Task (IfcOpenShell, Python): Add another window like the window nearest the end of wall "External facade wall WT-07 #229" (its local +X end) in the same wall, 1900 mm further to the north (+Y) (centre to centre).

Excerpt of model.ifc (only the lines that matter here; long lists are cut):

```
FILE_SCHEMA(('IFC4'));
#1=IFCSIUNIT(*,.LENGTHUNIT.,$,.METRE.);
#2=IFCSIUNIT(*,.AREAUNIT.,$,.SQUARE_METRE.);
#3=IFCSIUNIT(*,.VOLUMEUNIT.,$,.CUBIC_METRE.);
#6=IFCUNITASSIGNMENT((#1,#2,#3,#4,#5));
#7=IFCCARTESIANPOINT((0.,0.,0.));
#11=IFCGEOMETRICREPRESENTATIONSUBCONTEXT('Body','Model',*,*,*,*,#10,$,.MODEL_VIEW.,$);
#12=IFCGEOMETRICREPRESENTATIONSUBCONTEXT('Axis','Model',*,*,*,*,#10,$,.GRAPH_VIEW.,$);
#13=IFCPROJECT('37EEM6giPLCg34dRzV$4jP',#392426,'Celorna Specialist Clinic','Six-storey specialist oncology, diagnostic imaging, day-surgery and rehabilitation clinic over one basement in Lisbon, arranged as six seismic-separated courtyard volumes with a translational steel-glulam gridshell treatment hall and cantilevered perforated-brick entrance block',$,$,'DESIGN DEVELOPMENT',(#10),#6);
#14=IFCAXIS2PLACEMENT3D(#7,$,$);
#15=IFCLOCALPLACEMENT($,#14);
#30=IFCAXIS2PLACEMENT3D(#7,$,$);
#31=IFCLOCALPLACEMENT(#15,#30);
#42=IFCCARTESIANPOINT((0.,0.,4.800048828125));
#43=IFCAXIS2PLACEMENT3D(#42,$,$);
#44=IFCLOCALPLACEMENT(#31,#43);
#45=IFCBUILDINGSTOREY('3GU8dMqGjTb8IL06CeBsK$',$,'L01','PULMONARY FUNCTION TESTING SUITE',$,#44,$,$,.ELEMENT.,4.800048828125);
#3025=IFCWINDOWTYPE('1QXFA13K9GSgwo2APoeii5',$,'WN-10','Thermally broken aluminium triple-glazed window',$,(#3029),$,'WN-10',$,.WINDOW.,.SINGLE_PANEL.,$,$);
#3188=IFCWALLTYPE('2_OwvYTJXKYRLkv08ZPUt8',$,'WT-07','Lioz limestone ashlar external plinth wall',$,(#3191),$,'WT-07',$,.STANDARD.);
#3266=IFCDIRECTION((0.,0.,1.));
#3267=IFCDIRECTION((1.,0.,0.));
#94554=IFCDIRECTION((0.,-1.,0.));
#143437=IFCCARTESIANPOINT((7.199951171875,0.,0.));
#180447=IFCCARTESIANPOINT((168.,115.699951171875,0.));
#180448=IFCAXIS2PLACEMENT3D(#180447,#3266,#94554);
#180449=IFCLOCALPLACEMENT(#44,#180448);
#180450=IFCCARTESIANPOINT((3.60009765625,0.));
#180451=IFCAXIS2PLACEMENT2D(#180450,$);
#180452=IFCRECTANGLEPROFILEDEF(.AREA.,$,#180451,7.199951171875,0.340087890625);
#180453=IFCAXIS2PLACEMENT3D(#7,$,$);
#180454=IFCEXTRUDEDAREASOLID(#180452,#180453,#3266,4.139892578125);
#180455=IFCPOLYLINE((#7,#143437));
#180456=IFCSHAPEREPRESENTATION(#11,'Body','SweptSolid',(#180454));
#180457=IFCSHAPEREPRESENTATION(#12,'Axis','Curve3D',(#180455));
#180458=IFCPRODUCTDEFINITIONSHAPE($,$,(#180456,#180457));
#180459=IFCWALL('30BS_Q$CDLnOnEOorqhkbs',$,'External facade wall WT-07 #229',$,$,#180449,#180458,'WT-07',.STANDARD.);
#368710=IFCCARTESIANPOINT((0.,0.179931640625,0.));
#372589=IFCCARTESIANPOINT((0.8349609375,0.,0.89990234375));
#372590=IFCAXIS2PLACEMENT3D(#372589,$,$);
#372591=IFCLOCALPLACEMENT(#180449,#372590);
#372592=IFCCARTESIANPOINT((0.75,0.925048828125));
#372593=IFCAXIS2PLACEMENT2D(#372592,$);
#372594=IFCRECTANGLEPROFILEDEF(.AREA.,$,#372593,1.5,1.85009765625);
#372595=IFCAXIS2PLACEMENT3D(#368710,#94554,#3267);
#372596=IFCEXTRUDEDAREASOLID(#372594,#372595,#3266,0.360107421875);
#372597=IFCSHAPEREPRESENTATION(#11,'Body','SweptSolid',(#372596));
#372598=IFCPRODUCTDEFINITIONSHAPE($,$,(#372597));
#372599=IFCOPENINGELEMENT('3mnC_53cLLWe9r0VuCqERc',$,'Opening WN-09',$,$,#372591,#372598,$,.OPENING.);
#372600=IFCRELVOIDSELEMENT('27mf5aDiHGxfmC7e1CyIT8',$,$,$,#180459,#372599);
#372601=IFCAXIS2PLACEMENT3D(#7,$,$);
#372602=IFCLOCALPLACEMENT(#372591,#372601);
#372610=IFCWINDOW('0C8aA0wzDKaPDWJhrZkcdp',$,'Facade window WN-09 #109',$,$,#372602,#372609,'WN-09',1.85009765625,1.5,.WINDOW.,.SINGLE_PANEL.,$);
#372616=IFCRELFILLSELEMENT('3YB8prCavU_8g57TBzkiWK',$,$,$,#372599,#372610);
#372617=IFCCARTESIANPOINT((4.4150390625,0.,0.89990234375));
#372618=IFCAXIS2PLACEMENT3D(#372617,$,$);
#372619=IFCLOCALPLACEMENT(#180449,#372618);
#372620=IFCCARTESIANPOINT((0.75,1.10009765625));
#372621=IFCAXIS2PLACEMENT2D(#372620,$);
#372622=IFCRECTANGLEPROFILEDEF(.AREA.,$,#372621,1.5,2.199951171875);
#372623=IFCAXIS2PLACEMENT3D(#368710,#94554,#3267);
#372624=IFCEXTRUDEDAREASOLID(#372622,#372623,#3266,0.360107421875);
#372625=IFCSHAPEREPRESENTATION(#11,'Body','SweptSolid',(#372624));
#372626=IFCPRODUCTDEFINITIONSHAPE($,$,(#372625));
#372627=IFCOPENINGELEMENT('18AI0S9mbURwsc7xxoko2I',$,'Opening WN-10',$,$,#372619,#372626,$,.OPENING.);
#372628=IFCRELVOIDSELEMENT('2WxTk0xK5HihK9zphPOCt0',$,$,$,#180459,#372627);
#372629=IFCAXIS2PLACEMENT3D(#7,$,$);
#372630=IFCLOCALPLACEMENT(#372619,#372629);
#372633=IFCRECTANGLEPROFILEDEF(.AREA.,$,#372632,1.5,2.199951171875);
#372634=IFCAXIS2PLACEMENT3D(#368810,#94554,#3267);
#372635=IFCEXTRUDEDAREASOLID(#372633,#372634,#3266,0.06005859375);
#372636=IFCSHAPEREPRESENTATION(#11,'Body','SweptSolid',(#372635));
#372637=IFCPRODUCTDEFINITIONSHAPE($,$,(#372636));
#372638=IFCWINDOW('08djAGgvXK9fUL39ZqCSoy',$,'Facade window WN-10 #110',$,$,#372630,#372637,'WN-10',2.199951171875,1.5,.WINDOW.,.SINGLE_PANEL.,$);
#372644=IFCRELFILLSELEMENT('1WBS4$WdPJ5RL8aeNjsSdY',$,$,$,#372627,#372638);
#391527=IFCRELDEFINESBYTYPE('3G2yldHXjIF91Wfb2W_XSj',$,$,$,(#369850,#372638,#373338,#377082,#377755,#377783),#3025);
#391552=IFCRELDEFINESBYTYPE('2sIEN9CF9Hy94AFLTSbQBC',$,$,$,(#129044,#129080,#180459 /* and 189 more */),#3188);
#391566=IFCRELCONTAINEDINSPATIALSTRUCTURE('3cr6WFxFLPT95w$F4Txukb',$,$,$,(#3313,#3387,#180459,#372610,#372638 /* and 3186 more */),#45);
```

```python
import ifcopenshell
import ifcopenshell.api.feature
import ifcopenshell.api.geometry
import ifcopenshell.api.root
import ifcopenshell.geom
import ifcopenshell.util.element
import ifcopenshell.util.placement
import ifcopenshell.util.shape
import ifcopenshell.util.unit

model = ifcopenshell.open("model.ifc")
unit_scale = ifcopenshell.util.unit.calculate_unit_scale(model)
settings = ifcopenshell.geom.settings()


def volume(element):
    """Net volume in cubic metres, openings subtracted."""
    shape = ifcopenshell.geom.create_shape(settings, element)
    return ifcopenshell.util.shape.get_volume(shape.geometry)


window = model.by_guid("08djAGgvXK9fUL39ZqCSoy")
opening = window.FillsVoids[0].RelatingOpeningElement
wall = opening.VoidsElements[0].RelatingBuildingElement
before = volume(wall)
shift = ifcopenshell.util.placement.get_local_placement(wall.ObjectPlacement)[:3, 0] * -1.9 / unit_scale

# copy_class copies the void relationship, type, container and properties, but no geometry.
new_opening = ifcopenshell.api.root.copy_class(model, product=opening)
new_opening.Representation = ifcopenshell.util.element.copy_deep(
    model, opening.Representation, exclude=["IfcGeometricRepresentationContext", "IfcRepresentationMap"]
)
new_window = ifcopenshell.api.root.copy_class(model, product=window)
new_window.Representation = ifcopenshell.util.element.copy_deep(
    model, window.Representation, exclude=["IfcGeometricRepresentationContext", "IfcRepresentationMap"]
)
new_window.Tag = None
ifcopenshell.api.feature.add_filling(model, opening=new_opening, element=new_window)

for old, new in ((opening, new_opening), (window, new_window)):
    matrix = ifcopenshell.util.placement.get_local_placement(old.ObjectPlacement)
    matrix[:3, 3] += shift
    ifcopenshell.api.geometry.edit_object_placement(model, product=new, matrix=matrix, is_si=False)

after = volume(wall)

print(f"wall volume {before:.3f} -> {after:.3f} m3")

model.write("model_edited.ifc")
```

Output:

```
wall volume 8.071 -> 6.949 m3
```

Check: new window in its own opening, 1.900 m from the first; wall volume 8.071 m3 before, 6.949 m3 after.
